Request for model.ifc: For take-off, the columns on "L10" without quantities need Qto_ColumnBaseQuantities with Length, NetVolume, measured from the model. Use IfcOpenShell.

First a look at what the model holds.

```python
import ifcopenshell
import ifcopenshell.util.element
import ifcopenshell.util.unit

model = ifcopenshell.open("model.ifc")
print(model.schema)
for unit_type in ("LENGTHUNIT", "AREAUNIT", "VOLUMEUNIT"):
    print(unit_type, ifcopenshell.util.unit.calculate_unit_scale(model, unit_type))
storey = next(s for s in model.by_type("IfcBuildingStorey") if s.Name == "L10")
columns = [e for e in ifcopenshell.util.element.get_decomposition(storey) if e.is_a("IfcColumn")]
for e in sorted(columns, key=lambda e: e.id()):
    print(e.id(), e.is_a(), e.Name, list(ifcopenshell.util.element.get_psets(e, qtos_only=True)), sep=" | ")
```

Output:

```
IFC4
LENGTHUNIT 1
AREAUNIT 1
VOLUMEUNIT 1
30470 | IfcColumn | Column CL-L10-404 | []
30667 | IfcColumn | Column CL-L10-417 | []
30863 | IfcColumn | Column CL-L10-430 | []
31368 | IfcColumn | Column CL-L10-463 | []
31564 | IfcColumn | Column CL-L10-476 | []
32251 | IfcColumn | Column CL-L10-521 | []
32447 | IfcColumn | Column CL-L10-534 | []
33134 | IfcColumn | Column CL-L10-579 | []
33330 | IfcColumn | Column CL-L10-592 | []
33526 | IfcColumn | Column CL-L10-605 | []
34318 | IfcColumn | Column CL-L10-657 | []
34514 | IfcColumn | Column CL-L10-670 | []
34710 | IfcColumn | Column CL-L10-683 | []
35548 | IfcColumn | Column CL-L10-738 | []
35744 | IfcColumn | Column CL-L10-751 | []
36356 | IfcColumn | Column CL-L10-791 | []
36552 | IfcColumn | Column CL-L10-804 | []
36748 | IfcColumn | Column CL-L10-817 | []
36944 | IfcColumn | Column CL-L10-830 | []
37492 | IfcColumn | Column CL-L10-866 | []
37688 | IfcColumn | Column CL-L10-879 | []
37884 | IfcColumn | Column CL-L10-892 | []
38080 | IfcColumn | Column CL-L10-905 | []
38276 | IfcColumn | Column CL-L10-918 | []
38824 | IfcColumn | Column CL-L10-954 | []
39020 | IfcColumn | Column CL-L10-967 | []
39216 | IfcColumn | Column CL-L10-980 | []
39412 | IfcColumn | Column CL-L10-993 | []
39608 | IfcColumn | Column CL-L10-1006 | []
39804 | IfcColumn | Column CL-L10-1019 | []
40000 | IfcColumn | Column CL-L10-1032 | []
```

```python
import ifcopenshell
import ifcopenshell.api.pset
import ifcopenshell.geom
import ifcopenshell.util.element
import ifcopenshell.util.shape
import ifcopenshell.util.unit

model = ifcopenshell.open("model.ifc")
unit_scale = ifcopenshell.util.unit.calculate_unit_scale(model)
volume_scale = ifcopenshell.util.unit.calculate_unit_scale(model, "VOLUMEUNIT")
settings = ifcopenshell.geom.settings()

storey = next(s for s in model.by_type("IfcBuildingStorey") if s.Name == "L10")
columns = [e for e in ifcopenshell.util.element.get_decomposition(storey) if e.is_a("IfcColumn")]

for e in sorted(columns, key=lambda e: e.id()):
    if ifcopenshell.util.element.get_psets(e, qtos_only=True, should_inherit=False):
        continue
    # Geometry comes back in metres, in the element's own axes.
    shape = ifcopenshell.geom.create_shape(settings, e)
    values = {
        "Length": ifcopenshell.util.shape.get_z(shape.geometry) / unit_scale,
        "NetVolume": ifcopenshell.util.shape.get_volume(shape.geometry) / volume_scale,
    }
    qto = ifcopenshell.api.pset.add_qto(model, product=e, name="Qto_ColumnBaseQuantities")
    ifcopenshell.api.pset.edit_qto(model, qto=qto, properties=values)
    print(e.id(), {k: round(v, 3) for k, v in values.items()})

model.write("model_v2.ifc")
```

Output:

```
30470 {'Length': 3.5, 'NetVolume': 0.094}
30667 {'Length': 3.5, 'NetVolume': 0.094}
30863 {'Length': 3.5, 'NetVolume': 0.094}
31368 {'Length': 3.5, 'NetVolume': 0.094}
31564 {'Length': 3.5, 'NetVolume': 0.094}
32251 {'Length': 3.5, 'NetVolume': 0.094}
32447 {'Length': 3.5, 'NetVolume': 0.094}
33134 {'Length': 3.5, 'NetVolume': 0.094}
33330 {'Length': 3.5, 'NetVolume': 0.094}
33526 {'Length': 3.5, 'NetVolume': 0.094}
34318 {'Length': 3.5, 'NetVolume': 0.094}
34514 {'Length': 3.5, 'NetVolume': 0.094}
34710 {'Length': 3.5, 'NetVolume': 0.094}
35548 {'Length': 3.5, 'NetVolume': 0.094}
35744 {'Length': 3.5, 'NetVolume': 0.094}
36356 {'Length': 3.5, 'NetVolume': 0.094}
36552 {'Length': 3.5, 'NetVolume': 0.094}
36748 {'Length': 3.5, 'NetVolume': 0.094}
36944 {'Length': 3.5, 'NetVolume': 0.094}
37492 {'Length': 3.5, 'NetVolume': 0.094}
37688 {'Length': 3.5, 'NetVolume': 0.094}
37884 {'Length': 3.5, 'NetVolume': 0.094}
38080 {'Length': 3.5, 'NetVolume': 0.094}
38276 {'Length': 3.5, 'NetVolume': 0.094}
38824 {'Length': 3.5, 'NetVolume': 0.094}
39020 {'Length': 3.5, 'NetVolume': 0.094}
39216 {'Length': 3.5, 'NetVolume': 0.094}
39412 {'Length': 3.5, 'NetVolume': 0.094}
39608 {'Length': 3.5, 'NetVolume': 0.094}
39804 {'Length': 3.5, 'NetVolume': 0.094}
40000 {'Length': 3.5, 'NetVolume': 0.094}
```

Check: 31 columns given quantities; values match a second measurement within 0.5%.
